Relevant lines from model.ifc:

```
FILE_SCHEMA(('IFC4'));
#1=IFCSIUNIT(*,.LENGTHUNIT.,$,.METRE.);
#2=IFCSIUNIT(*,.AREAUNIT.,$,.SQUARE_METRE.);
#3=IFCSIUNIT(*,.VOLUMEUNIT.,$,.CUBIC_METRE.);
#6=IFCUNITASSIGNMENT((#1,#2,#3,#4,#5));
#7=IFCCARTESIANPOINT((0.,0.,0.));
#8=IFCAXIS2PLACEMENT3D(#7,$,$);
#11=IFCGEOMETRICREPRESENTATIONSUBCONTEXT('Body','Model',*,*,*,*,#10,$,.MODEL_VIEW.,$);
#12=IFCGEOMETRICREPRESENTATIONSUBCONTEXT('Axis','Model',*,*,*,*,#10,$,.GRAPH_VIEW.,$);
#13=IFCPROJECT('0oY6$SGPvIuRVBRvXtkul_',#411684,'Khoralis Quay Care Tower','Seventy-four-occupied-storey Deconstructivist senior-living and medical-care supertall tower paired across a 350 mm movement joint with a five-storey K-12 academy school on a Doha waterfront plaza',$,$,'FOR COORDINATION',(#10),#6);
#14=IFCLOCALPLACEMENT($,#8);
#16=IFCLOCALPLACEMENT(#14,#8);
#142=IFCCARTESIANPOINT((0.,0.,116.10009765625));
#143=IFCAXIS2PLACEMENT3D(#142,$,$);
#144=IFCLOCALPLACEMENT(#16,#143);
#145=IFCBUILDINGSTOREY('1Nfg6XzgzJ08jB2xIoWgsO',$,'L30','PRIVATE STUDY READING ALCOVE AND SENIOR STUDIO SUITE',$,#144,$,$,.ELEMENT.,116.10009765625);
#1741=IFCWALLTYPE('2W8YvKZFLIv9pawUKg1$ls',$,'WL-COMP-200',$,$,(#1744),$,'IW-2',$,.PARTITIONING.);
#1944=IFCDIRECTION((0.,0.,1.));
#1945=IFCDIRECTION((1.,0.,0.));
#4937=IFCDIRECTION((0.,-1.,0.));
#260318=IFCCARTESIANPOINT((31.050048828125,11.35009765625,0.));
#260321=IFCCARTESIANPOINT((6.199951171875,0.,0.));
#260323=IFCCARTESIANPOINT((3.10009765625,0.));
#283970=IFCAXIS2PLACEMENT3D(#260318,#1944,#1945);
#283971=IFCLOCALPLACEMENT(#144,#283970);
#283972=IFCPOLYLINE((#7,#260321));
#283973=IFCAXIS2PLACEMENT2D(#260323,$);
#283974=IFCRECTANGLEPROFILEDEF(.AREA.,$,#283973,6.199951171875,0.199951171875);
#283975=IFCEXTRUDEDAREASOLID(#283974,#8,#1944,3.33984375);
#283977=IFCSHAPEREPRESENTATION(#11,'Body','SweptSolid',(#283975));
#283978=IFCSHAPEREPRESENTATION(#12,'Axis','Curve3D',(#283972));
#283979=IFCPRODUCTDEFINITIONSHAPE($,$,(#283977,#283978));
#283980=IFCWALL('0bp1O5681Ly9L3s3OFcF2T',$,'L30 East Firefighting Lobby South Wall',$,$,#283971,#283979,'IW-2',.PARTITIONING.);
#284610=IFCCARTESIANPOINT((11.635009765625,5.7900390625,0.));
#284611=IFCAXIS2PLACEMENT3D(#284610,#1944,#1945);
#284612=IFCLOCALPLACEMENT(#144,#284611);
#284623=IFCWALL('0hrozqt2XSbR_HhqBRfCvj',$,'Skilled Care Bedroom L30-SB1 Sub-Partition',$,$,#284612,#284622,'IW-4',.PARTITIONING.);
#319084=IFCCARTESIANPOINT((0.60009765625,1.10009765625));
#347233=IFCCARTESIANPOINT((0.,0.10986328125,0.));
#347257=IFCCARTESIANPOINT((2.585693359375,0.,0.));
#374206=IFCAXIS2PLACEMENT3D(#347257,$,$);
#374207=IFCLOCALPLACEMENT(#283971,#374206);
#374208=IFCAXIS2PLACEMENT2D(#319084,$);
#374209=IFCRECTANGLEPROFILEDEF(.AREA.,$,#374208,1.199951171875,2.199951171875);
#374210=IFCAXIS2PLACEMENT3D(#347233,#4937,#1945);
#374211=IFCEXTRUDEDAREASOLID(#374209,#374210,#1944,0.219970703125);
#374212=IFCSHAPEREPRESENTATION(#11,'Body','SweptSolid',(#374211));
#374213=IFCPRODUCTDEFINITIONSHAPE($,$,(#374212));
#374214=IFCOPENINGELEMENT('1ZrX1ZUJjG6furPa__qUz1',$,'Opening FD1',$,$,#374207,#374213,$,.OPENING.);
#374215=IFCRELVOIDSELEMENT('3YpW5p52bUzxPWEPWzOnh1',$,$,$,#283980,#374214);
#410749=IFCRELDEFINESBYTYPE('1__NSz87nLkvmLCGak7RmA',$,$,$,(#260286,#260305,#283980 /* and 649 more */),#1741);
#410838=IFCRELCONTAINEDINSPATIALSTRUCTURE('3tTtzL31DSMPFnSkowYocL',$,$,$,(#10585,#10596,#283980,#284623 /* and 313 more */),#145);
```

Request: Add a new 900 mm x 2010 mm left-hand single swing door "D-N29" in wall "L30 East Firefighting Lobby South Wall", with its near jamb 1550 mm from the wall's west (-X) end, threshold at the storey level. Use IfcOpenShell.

```python
import numpy as np
import ifcopenshell
import ifcopenshell.api.feature
import ifcopenshell.api.geometry
import ifcopenshell.api.root
import ifcopenshell.api.spatial
import ifcopenshell.geom
import ifcopenshell.util.element
import ifcopenshell.util.placement
import ifcopenshell.util.representation
import ifcopenshell.util.shape
import ifcopenshell.util.unit

model = ifcopenshell.open("model.ifc")
unit_scale = ifcopenshell.util.unit.calculate_unit_scale(model)
settings = ifcopenshell.geom.settings()


def volume(element):
    """Net volume in cubic metres, openings subtracted."""
    shape = ifcopenshell.geom.create_shape(settings, element)
    return ifcopenshell.util.shape.get_volume(shape.geometry)


wall = model.by_guid("0bp1O5681Ly9L3s3OFcF2T")
storey = ifcopenshell.util.element.get_container(wall, ifc_class="IfcBuildingStorey")
context = ifcopenshell.util.representation.get_context(model, "Model", "Body", "MODEL_VIEW")
before = volume(wall)

width, height, from_end, sill = 0.9, 2.01, 1.55, 0.0  # metres

# The wall runs along its own X axis, and the end named is its -X end.
wall_shape = ifcopenshell.geom.create_shape(settings, wall)
x, y, z = ifcopenshell.util.shape.get_vertices(wall_shape.geometry).T
start = x.min() + from_end
face, thickness = float(y.min()), float(y.max() - y.min())
wall_matrix = ifcopenshell.util.placement.get_local_placement(wall.ObjectPlacement)
level = ifcopenshell.util.placement.get_local_placement(storey.ObjectPlacement)[2, 3]


def in_wall(x, y):
    """Placement at x, y metres in the wall's axes, at sill height."""
    matrix = wall_matrix.copy()
    matrix[:, 3] = wall_matrix @ np.array([x / unit_scale, y / unit_scale, 0.0, 1.0])
    matrix[2, 3] = level + sill / unit_scale
    return matrix


# Opening: a box that overshoots both wall faces by 50 mm.
opening = ifcopenshell.api.root.create_entity(model, ifc_class="IfcOpeningElement", predefined_type="OPENING")
box = ifcopenshell.api.geometry.add_wall_representation(
    model, context=context, length=width, height=height, thickness=thickness + 0.1
)
ifcopenshell.api.geometry.assign_representation(model, product=opening, representation=box)
ifcopenshell.api.geometry.edit_object_placement(model, product=opening, matrix=in_wall(start, face - 0.05), is_si=False)
ifcopenshell.api.feature.add_feature(model, feature=opening, element=wall)

door = ifcopenshell.api.root.create_entity(model, ifc_class="IfcDoor", name="D-N29", predefined_type="DOOR")
door.OverallWidth, door.OverallHeight = width / unit_scale, height / unit_scale
door.OperationType = "SINGLE_SWING_LEFT"
body = ifcopenshell.api.geometry.add_door_representation(
    model,
    context=context,
    overall_width=door.OverallWidth,
    overall_height=door.OverallHeight,
    operation_type="SINGLE_SWING_LEFT",
    lining_properties={"LiningDepth": thickness / unit_scale, "ThresholdDepth": thickness / unit_scale},
)
ifcopenshell.api.geometry.assign_representation(model, product=door, representation=body)
ifcopenshell.api.spatial.assign_container(model, products=[door], relating_structure=storey)
ifcopenshell.api.feature.add_filling(model, opening=opening, element=door)

# The lining spans the wall, so the door starts at the wall face.
ifcopenshell.api.geometry.edit_object_placement(model, product=door, matrix=in_wall(start, face), is_si=False)

after = volume(wall)

print(f"wall volume {before:.3f} -> {after:.3f} m3")

model.write("model_updated.ifc")
```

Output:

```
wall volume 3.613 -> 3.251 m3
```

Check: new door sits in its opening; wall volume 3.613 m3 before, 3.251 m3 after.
